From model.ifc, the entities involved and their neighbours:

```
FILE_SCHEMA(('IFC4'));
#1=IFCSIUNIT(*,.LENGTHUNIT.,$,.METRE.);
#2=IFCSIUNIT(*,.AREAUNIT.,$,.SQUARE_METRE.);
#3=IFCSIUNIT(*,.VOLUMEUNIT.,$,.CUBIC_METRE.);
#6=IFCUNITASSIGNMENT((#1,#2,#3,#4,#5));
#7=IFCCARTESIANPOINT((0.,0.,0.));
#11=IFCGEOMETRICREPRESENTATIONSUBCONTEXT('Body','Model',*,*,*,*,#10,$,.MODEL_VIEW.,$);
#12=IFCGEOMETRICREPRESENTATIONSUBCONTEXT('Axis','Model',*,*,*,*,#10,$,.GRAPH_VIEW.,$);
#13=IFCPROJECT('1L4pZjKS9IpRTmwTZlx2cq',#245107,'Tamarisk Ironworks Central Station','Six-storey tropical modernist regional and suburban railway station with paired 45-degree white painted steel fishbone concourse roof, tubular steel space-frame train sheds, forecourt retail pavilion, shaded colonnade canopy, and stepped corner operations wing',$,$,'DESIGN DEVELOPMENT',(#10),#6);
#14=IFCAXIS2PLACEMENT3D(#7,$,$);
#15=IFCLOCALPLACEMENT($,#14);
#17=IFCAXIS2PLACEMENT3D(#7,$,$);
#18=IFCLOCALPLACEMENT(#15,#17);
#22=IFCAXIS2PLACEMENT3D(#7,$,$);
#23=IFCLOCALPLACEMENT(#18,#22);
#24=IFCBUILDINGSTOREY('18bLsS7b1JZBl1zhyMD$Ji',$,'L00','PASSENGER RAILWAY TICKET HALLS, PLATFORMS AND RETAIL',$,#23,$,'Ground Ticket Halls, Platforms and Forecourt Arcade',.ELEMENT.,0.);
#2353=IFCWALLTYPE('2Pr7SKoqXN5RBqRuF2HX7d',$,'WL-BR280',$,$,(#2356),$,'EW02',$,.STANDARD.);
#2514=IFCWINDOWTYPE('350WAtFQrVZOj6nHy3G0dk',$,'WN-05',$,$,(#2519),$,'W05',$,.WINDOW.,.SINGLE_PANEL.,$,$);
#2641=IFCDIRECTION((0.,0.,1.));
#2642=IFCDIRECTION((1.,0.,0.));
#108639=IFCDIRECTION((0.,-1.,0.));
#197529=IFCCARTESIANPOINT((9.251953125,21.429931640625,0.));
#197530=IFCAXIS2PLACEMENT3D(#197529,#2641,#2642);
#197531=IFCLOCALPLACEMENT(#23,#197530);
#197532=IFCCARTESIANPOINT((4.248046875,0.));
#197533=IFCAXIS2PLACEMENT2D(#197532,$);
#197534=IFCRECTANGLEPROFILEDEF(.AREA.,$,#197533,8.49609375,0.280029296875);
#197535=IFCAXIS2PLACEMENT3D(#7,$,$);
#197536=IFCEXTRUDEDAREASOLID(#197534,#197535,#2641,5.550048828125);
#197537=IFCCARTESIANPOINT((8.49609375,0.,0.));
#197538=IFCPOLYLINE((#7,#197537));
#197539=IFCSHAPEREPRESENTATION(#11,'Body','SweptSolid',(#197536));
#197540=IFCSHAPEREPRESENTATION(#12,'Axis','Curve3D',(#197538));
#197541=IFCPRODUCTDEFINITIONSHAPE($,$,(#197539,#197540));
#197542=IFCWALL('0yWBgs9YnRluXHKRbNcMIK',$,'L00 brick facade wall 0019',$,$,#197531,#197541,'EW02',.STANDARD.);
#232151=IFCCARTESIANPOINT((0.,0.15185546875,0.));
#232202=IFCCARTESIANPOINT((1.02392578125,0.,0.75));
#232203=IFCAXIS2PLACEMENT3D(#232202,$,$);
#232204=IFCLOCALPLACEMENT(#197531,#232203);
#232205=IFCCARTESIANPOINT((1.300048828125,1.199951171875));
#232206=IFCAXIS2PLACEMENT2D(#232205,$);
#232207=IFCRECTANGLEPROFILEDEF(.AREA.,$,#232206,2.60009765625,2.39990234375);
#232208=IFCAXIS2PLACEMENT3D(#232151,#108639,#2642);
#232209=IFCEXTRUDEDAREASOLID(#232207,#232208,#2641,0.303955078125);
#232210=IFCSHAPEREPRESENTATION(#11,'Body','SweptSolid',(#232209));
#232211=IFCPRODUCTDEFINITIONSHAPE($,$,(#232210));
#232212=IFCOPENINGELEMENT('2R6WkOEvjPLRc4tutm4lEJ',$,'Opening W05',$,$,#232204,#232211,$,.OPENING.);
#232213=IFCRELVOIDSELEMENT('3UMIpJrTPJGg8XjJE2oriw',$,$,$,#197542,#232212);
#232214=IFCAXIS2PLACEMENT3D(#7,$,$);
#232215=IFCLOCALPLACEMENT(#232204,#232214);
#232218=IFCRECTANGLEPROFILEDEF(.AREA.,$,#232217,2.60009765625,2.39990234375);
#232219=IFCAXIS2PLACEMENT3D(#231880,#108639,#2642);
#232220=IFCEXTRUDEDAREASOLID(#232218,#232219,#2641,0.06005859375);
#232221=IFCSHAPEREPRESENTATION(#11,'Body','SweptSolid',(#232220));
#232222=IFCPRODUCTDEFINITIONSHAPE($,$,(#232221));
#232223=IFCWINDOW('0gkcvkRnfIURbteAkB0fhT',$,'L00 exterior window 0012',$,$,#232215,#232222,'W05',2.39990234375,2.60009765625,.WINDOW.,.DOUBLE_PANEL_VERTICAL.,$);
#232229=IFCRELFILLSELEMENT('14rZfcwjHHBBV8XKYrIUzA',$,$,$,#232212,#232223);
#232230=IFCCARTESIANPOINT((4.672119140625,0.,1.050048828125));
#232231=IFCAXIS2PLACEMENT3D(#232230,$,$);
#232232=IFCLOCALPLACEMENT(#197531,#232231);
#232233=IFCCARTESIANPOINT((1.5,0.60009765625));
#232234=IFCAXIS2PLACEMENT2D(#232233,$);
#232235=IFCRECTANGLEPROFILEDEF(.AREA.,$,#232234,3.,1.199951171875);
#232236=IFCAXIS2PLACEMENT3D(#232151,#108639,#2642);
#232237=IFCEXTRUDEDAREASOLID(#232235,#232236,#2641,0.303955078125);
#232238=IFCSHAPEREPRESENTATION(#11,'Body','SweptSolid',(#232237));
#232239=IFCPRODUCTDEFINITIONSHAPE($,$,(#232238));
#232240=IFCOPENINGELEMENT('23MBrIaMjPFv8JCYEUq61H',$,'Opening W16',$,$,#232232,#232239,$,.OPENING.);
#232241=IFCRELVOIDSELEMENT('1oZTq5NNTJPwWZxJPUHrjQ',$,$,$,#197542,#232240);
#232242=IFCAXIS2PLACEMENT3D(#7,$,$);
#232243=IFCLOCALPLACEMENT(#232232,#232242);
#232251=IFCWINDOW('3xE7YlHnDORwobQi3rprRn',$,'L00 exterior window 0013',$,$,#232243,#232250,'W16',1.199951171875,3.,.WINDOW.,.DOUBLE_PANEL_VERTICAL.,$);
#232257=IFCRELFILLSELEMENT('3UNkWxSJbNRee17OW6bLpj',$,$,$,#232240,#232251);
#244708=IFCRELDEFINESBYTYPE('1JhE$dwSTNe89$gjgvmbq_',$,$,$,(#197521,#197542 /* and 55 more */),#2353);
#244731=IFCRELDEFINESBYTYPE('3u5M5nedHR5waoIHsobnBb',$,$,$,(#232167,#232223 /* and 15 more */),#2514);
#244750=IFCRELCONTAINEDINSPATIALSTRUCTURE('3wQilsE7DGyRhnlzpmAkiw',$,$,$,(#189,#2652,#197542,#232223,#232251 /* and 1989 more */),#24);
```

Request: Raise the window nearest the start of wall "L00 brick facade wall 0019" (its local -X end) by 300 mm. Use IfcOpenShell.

```python
import numpy as np
import ifcopenshell
import ifcopenshell.api.geometry
import ifcopenshell.util.placement
import ifcopenshell.util.unit

model = ifcopenshell.open("model.ifc")
unit_scale = ifcopenshell.util.unit.calculate_unit_scale(model)

window = model.by_id(232223)
opening = window.FillsVoids[0].RelatingOpeningElement
dz = 0.3 / unit_scale

shift = np.array([0.0, 0.0, dz])
# The window is placed relative to its opening, so it follows when the opening moves.
matrix = ifcopenshell.util.placement.get_local_placement(opening.ObjectPlacement)
matrix[:3, 3] += shift
ifcopenshell.api.geometry.edit_object_placement(
    model, product=opening, matrix=matrix, is_si=False, should_transform_children=True
)

print(f"moved by {dz * unit_scale:+.3f} m")

model.write("model-out.ifc")
```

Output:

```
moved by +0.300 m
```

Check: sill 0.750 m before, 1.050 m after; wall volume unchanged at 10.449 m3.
